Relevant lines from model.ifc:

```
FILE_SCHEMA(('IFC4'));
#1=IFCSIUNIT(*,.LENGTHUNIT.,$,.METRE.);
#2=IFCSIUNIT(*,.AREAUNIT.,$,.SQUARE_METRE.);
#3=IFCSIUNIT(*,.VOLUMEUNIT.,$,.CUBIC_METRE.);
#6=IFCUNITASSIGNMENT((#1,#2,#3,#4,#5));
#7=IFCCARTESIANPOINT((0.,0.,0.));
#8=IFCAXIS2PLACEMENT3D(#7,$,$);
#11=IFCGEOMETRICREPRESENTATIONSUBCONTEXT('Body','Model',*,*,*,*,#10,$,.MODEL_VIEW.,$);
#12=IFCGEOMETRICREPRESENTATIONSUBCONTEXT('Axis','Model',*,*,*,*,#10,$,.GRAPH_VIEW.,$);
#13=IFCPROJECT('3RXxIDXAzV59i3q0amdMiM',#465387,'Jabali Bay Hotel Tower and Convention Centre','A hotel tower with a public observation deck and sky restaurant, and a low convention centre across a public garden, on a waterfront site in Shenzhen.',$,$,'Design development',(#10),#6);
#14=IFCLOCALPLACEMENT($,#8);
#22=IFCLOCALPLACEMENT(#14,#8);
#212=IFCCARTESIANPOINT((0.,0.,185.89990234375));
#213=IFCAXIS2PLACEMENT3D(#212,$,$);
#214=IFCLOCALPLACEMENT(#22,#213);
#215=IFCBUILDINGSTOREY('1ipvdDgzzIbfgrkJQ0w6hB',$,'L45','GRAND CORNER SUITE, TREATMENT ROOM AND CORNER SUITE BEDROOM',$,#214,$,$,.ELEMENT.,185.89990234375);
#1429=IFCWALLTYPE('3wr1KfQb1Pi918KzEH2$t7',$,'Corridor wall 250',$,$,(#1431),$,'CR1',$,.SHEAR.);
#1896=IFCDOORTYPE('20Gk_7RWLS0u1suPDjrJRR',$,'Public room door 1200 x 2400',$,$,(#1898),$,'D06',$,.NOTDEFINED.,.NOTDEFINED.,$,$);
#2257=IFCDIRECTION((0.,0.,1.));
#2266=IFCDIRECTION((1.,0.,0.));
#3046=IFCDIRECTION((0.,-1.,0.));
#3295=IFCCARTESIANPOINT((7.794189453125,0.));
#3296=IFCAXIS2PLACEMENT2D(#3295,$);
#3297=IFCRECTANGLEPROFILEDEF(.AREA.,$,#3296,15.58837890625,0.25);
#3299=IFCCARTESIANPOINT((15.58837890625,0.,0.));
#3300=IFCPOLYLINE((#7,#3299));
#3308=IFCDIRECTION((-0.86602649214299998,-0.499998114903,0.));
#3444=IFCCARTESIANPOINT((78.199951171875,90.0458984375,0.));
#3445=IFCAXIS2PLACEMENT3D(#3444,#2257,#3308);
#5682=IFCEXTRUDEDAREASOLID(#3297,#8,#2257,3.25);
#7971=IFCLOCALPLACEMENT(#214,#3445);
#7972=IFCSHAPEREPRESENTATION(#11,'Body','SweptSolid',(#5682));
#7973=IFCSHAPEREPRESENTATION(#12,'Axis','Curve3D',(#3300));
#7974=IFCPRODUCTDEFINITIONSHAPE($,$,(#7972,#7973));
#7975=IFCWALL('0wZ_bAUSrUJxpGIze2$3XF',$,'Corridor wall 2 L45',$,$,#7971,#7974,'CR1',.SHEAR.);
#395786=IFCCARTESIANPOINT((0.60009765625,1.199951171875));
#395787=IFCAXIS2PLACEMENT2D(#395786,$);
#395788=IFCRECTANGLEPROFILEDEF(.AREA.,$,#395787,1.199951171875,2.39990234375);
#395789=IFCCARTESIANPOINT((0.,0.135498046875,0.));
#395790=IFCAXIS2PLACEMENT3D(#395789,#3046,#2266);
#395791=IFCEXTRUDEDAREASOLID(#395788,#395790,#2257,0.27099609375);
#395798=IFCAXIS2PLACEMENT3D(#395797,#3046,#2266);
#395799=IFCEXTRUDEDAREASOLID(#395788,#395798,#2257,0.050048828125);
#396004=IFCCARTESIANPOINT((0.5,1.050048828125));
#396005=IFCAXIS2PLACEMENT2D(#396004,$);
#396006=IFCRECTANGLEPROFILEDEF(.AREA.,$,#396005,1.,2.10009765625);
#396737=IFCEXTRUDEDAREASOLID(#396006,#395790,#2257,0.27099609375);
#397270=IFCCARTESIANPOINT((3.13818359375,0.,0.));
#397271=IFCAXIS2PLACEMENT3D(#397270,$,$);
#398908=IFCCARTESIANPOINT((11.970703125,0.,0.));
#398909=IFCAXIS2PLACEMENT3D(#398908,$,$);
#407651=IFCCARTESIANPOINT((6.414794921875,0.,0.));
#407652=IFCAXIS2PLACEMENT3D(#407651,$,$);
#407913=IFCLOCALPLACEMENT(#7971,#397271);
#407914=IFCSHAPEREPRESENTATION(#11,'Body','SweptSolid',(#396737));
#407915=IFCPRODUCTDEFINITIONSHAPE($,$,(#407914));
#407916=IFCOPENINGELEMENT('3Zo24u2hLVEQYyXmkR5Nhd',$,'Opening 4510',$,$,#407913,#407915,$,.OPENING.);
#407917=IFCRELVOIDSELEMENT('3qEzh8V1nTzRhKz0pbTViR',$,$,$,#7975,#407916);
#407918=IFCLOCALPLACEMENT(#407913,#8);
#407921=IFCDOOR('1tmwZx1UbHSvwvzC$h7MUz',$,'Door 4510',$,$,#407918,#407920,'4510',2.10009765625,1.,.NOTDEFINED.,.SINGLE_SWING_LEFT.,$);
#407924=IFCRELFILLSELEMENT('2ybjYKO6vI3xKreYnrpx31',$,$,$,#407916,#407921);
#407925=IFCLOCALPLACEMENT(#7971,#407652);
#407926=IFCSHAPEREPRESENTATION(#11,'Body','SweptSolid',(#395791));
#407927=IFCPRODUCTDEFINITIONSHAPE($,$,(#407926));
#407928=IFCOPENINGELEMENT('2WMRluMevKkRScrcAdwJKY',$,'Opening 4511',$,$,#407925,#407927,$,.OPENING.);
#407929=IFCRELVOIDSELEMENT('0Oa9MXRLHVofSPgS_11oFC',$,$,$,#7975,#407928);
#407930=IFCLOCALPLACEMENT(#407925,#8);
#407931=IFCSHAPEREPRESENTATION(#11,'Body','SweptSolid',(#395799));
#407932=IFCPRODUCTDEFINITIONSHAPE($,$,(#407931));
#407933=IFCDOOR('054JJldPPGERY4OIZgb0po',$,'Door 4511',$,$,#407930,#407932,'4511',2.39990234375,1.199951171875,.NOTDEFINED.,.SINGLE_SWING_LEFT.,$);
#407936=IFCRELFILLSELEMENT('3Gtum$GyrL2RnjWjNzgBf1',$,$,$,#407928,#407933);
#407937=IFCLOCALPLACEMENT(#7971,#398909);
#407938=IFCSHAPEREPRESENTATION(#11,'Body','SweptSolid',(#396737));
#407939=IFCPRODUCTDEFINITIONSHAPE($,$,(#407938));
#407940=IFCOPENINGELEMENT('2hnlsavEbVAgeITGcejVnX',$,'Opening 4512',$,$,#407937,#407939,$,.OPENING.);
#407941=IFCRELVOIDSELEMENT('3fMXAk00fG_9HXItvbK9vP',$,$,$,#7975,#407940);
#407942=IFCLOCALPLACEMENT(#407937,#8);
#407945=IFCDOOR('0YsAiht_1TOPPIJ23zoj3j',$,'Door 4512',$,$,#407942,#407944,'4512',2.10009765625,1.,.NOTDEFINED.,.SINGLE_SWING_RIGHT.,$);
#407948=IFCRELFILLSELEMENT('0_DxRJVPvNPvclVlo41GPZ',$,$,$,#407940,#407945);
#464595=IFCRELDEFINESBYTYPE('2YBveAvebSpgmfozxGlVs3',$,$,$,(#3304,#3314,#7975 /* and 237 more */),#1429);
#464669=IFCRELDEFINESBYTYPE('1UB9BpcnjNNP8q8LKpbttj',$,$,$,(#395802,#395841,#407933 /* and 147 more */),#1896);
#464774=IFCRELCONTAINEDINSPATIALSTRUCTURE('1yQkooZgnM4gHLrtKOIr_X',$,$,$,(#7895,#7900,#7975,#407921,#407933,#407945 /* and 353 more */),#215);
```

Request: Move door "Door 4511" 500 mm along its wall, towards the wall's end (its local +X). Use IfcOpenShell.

```python
import ifcopenshell
import ifcopenshell.api.geometry
import ifcopenshell.util.placement

model = ifcopenshell.open("model.ifc")

door = model.by_guid("054JJldPPGERY4OIZgb0po")
opening = door.FillsVoids[0].RelatingOpeningElement
wall = opening.VoidsElements[0].RelatingBuildingElement

wall_matrix = ifcopenshell.util.placement.get_local_placement(wall.ObjectPlacement)
shift = wall_matrix[:3, 0] * 0.5
before = ifcopenshell.util.placement.get_local_placement(door.ObjectPlacement)[:3, 3].copy()

# The door is placed relative to its opening, so it follows when the opening moves.
matrix = ifcopenshell.util.placement.get_local_placement(opening.ObjectPlacement)
matrix[:3, 3] += shift
ifcopenshell.api.geometry.edit_object_placement(
    model, product=opening, matrix=matrix, is_si=False, should_transform_children=True
)

after = ifcopenshell.util.placement.get_local_placement(door.ObjectPlacement)[:3, 3]
print("door moved by", (after - before).round(3) + 0.0)

model.write("model-out.ifc")
```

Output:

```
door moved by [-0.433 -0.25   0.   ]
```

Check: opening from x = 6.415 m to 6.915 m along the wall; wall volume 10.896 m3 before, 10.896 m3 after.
